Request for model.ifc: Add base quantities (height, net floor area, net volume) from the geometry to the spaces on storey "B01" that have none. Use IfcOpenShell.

First a look at what the model holds.

```python
import ifcopenshell
import ifcopenshell.util.element
import ifcopenshell.util.unit

model = ifcopenshell.open("model.ifc")
print(model.schema)
for unit_type in ("LENGTHUNIT", "AREAUNIT", "VOLUMEUNIT"):
    print(unit_type, ifcopenshell.util.unit.calculate_unit_scale(model, unit_type))
storey = next(s for s in model.by_type("IfcBuildingStorey") if s.Name == "B01")
spaces = [e for e in ifcopenshell.util.element.get_decomposition(storey) if e.is_a("IfcSpace")]
for e in sorted(spaces, key=lambda e: e.id()):
    print(e.id(), e.is_a(), e.Name, list(ifcopenshell.util.element.get_psets(e, qtos_only=True)), sep=" | ")
```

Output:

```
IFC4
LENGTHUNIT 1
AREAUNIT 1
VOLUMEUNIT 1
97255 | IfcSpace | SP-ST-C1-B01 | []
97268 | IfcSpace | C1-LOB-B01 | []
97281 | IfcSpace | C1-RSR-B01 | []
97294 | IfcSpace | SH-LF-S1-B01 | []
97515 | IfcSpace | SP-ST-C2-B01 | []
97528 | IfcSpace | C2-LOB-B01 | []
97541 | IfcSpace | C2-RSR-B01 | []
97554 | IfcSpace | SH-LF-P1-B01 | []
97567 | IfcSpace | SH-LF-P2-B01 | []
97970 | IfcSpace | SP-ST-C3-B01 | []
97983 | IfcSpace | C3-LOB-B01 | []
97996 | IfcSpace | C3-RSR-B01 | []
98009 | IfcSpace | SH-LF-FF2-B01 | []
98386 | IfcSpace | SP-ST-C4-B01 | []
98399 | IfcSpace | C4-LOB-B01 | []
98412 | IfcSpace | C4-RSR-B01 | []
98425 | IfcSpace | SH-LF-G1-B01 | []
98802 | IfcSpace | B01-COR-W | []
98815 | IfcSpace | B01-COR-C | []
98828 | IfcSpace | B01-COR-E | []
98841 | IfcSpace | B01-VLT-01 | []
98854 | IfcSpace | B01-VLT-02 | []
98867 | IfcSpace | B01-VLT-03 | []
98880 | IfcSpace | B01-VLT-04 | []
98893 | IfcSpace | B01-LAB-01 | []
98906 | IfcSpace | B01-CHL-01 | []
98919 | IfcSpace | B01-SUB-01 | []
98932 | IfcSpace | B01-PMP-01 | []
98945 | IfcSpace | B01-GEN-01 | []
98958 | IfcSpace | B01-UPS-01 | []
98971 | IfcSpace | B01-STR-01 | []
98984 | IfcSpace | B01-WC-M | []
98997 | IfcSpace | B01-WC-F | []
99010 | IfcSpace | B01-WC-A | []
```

```python
import ifcopenshell
import ifcopenshell.api.pset
import ifcopenshell.geom
import ifcopenshell.util.element
import ifcopenshell.util.shape
import ifcopenshell.util.unit

model = ifcopenshell.open("model.ifc")
unit_scale = ifcopenshell.util.unit.calculate_unit_scale(model)
area_scale = ifcopenshell.util.unit.calculate_unit_scale(model, "AREAUNIT")
volume_scale = ifcopenshell.util.unit.calculate_unit_scale(model, "VOLUMEUNIT")
settings = ifcopenshell.geom.settings()

storey = next(s for s in model.by_type("IfcBuildingStorey") if s.Name == "B01")
spaces = [e for e in ifcopenshell.util.element.get_decomposition(storey) if e.is_a("IfcSpace")]

for e in sorted(spaces, key=lambda e: e.id()):
    if ifcopenshell.util.element.get_psets(e, qtos_only=True, should_inherit=False):
        continue
    # Geometry comes back in metres, in the element's own axes.
    shape = ifcopenshell.geom.create_shape(settings, e)
    values = {
        "Height": ifcopenshell.util.shape.get_z(shape.geometry) / unit_scale,
        "NetFloorArea": ifcopenshell.util.shape.get_footprint_area(shape.geometry) / area_scale,
        "NetVolume": ifcopenshell.util.shape.get_volume(shape.geometry) / volume_scale,
    }
    qto = ifcopenshell.api.pset.add_qto(model, product=e, name="Qto_SpaceBaseQuantities")
    ifcopenshell.api.pset.edit_qto(model, qto=qto, properties=values)
    print(e.id(), {k: round(v, 3) for k, v in values.items()})

model.write("model_rev.ifc")
```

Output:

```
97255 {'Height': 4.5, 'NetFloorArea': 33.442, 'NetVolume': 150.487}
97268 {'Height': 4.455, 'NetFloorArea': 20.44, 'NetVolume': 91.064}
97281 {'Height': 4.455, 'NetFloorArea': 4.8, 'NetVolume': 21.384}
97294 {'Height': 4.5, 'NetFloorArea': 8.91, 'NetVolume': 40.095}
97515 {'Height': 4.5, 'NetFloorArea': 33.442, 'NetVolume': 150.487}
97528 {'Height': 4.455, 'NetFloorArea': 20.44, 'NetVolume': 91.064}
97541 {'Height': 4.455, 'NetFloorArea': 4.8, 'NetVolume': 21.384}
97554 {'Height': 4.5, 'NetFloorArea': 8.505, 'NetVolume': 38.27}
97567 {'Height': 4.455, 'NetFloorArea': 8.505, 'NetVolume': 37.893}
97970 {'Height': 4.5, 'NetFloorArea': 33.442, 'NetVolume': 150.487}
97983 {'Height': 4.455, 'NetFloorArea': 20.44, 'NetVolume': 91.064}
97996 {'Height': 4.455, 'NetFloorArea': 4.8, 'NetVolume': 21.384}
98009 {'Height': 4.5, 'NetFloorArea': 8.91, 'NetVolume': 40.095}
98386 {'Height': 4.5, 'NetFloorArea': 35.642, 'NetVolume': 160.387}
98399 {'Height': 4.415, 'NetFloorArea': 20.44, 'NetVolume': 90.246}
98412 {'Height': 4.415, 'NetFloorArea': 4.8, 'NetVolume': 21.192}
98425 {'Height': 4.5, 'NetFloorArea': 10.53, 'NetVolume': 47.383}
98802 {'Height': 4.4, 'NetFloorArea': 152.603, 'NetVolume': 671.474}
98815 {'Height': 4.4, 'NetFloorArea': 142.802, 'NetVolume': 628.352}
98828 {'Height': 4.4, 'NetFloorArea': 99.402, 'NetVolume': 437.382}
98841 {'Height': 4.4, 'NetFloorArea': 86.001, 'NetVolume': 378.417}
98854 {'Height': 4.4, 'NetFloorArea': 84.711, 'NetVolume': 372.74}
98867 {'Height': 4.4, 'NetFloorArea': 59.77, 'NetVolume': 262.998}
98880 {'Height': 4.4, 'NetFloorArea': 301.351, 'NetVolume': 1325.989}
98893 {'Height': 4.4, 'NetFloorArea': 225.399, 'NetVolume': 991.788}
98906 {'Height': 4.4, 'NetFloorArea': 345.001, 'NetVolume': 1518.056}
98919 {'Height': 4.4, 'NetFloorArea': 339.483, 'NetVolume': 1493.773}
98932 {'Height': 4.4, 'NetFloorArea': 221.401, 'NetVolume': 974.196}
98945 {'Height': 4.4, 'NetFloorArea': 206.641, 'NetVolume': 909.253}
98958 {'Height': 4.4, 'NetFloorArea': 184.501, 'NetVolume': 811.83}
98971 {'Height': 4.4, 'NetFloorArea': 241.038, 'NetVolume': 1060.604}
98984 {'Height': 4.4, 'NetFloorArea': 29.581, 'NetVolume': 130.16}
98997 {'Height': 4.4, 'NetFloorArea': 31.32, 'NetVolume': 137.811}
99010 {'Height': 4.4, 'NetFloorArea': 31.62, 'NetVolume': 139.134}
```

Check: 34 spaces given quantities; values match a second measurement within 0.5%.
